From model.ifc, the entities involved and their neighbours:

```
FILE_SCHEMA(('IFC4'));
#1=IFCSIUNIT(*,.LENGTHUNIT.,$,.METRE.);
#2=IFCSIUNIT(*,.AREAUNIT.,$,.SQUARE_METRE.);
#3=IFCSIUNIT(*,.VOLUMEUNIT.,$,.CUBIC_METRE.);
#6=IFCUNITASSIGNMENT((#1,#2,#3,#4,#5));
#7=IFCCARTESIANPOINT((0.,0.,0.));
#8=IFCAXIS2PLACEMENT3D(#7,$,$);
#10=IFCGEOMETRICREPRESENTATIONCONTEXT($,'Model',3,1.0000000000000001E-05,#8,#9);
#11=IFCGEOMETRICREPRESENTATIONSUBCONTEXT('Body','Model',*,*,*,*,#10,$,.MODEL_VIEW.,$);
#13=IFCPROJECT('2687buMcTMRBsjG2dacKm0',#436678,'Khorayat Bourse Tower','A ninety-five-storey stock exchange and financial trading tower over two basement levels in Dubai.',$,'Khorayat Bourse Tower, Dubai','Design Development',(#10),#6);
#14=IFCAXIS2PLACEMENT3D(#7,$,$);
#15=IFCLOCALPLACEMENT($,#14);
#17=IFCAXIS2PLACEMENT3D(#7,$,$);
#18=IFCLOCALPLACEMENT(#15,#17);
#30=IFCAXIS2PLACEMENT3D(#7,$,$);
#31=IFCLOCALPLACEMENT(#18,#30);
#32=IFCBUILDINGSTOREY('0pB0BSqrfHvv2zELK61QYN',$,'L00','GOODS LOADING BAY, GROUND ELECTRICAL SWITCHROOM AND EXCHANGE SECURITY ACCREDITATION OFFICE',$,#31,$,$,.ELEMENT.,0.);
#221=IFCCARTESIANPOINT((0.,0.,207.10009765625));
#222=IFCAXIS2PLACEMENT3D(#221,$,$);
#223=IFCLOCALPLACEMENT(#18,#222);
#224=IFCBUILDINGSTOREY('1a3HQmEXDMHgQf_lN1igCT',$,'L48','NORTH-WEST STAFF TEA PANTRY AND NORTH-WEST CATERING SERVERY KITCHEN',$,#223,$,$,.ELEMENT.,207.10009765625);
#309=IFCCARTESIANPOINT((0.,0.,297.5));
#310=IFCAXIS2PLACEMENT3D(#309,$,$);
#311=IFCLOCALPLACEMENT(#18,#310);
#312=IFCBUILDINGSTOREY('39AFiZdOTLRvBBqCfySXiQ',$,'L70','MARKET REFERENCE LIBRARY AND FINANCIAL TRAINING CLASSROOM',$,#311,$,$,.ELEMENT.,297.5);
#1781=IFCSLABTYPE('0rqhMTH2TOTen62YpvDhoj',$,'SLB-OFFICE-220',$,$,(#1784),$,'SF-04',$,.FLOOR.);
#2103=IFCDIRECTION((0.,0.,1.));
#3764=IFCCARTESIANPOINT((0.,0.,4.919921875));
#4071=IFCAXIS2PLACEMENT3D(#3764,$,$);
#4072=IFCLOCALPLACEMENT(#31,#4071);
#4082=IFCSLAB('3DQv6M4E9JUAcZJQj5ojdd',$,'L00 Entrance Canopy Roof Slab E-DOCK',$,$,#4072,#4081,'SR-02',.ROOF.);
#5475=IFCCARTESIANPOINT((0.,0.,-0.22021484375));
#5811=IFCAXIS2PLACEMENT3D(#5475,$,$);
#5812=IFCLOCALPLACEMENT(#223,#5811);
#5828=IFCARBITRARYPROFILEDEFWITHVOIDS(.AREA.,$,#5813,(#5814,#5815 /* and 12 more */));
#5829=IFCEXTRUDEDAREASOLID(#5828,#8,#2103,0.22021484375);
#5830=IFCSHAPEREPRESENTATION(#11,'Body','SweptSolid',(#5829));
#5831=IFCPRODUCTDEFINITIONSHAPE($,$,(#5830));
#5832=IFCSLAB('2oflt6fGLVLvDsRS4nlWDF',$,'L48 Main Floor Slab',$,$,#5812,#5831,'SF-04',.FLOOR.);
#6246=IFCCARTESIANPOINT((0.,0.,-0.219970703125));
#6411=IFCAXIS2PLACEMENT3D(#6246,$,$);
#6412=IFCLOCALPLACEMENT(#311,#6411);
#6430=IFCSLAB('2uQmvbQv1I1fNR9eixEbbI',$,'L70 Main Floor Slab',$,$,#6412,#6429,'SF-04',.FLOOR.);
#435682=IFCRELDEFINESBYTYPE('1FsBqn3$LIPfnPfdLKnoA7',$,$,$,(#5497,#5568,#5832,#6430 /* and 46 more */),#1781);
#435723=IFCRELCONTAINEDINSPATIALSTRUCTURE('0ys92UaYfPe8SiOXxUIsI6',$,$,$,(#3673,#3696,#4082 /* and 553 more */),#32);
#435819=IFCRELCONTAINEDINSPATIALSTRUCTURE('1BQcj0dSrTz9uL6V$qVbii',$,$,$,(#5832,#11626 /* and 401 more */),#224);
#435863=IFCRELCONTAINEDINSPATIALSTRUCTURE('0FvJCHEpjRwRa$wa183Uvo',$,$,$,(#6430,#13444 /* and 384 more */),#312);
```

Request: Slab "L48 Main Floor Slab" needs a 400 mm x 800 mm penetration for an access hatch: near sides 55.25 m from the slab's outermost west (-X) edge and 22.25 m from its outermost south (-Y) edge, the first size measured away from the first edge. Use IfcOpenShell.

```python
import numpy as np
import ifcopenshell
import ifcopenshell.api.feature
import ifcopenshell.api.geometry
import ifcopenshell.api.root
import ifcopenshell.geom
import ifcopenshell.util.placement
import ifcopenshell.util.representation
import ifcopenshell.util.shape
import ifcopenshell.util.unit

model = ifcopenshell.open("model.ifc")
unit_scale = ifcopenshell.util.unit.calculate_unit_scale(model)
settings = ifcopenshell.geom.settings()


def volume(element):
    """Net volume in cubic metres, openings subtracted."""
    shape = ifcopenshell.geom.create_shape(settings, element)
    return ifcopenshell.util.shape.get_volume(shape.geometry)


slab = model.by_guid("2oflt6fGLVLvDsRS4nlWDF")
before = volume(slab)

# Extent in the slab's own axes, in metres. The edges named are its -X and -Y sides.
slab_shape = ifcopenshell.geom.create_shape(settings, slab)
vertices = ifcopenshell.util.shape.get_vertices(slab_shape.geometry)
x_min, y_min, bottom = vertices.min(axis=0)
top = vertices[:, 2].max()

opening = ifcopenshell.api.root.create_entity(model, ifc_class="IfcOpeningElement", name="Access hatch opening", predefined_type="OPENING")
context = ifcopenshell.util.representation.get_context(model, "Model", "Body", "MODEL_VIEW")
width, depth = 0.4, 0.8
outline = [(0.0, 0.0), (width, 0.0), (width, depth), (0.0, depth), (0.0, 0.0)]
# Overshoot both faces by 50 mm so the cut is clean.
shape = ifcopenshell.api.geometry.add_slab_representation(
    model, context=context, depth=top - bottom + 0.1, polyline=outline
)
ifcopenshell.api.geometry.assign_representation(model, product=opening, representation=shape)

matrix = ifcopenshell.util.placement.get_local_placement(slab.ObjectPlacement)
matrix[:, 3] = matrix @ np.append(np.array([x_min + 55.25, y_min + 22.25, bottom - 0.05]) / unit_scale, 1.0)
ifcopenshell.api.geometry.edit_object_placement(model, product=opening, matrix=matrix, is_si=False)
ifcopenshell.api.feature.add_feature(model, feature=opening, element=slab)

after = volume(slab)

print(f"slab volume {before:.3f} -> {after:.3f} m3")

model.write("model_rev.ifc")
```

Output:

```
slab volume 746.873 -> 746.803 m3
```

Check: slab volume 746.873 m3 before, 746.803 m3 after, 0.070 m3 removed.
